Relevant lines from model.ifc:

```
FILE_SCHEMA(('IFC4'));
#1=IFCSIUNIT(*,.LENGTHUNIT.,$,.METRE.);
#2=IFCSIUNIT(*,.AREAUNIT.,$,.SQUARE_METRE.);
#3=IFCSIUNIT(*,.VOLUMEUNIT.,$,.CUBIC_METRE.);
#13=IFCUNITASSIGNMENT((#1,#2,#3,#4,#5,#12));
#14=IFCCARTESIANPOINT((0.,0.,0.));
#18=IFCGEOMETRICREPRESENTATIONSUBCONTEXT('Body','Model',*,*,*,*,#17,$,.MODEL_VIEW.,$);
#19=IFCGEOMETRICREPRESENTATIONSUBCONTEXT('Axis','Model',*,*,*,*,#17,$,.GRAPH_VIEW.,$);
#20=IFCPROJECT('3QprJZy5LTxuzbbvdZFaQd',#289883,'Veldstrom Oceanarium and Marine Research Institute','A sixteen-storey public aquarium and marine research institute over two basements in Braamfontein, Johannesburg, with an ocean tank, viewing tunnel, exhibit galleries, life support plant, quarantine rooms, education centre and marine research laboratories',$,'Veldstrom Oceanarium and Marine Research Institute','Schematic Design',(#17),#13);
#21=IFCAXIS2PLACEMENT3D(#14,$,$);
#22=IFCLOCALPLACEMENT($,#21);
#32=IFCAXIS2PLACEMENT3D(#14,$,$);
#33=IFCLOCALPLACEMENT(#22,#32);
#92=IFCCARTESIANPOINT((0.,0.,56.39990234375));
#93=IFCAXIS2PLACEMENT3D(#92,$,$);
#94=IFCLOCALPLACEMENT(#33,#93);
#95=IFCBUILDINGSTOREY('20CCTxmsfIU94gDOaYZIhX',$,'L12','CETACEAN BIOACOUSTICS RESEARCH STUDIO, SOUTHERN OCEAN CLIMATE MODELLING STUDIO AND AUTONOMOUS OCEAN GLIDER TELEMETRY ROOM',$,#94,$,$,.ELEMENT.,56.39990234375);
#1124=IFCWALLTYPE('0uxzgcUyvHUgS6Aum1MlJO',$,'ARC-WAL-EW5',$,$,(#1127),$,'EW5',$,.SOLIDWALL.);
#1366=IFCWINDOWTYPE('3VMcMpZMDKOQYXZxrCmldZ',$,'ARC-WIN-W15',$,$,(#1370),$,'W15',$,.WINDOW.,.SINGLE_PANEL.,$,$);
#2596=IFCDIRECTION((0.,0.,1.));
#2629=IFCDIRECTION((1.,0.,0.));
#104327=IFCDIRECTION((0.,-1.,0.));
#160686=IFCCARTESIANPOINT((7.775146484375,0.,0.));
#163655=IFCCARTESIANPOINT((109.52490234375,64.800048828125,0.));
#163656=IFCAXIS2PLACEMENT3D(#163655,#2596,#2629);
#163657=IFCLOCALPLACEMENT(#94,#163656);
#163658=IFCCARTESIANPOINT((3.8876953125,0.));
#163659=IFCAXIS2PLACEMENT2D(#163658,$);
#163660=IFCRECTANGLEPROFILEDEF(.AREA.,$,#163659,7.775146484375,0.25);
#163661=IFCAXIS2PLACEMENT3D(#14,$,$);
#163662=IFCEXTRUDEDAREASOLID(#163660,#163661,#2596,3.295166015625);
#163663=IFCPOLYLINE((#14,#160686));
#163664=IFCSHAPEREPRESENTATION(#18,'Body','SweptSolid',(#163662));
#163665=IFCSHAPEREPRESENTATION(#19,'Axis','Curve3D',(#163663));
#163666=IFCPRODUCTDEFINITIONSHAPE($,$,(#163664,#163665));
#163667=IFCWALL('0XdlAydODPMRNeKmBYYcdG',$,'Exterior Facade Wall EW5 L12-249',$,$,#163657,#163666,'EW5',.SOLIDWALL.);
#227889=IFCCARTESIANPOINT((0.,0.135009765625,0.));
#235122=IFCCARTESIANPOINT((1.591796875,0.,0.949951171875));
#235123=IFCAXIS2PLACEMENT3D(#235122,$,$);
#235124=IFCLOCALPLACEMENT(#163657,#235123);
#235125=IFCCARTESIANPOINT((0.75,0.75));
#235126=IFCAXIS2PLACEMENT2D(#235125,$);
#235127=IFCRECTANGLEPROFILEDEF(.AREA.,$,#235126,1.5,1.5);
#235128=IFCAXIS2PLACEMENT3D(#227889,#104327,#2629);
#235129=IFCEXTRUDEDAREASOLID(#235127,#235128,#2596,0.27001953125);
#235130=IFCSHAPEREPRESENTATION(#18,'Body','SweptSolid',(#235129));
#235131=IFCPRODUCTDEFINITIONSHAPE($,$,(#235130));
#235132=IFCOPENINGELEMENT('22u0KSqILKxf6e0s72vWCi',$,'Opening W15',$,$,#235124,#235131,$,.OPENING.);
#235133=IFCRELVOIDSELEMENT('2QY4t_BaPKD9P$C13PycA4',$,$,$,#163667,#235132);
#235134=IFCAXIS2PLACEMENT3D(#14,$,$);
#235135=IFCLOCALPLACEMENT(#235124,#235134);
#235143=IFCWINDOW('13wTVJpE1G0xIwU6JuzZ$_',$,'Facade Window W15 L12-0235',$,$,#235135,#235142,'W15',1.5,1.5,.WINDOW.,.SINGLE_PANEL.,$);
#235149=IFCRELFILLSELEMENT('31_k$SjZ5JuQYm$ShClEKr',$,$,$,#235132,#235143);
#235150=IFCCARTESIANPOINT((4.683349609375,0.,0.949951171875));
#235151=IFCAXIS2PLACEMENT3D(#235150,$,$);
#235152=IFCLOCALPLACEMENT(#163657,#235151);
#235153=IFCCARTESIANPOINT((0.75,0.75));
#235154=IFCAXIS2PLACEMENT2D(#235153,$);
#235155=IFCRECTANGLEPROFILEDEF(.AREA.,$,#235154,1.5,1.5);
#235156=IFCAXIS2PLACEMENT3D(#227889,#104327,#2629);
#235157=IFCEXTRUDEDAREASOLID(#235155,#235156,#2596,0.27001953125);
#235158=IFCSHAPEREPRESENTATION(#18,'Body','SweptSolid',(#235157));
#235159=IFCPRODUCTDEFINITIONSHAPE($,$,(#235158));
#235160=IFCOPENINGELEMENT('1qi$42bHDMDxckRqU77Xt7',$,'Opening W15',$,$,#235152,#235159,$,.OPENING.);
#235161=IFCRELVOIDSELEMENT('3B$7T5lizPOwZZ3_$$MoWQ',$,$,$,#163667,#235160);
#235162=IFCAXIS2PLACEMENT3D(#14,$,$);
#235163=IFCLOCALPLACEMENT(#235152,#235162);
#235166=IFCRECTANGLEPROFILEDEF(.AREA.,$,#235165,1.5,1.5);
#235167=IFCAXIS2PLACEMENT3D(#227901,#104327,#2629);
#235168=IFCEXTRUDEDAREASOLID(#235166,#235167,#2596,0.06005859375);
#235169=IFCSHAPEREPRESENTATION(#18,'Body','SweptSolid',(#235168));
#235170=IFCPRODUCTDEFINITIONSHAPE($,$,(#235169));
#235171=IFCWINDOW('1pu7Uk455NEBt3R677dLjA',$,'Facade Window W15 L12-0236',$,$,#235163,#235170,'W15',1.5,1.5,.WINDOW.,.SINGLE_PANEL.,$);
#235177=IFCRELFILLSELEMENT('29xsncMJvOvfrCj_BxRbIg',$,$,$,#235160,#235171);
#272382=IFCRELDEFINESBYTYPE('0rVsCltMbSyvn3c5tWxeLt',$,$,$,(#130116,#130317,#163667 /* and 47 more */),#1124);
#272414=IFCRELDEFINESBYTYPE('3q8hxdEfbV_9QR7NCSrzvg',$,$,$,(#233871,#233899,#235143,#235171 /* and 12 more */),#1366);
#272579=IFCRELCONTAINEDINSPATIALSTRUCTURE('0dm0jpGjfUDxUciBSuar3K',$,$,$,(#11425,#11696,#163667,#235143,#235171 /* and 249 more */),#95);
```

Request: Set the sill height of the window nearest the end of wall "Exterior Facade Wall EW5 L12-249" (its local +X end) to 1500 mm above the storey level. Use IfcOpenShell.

```python
import numpy as np
import ifcopenshell
import ifcopenshell.api.geometry
import ifcopenshell.geom
import ifcopenshell.util.element
import ifcopenshell.util.placement
import ifcopenshell.util.shape
import ifcopenshell.util.unit

model = ifcopenshell.open("model.ifc")
unit_scale = ifcopenshell.util.unit.calculate_unit_scale(model)

window = model.by_guid("1pu7Uk455NEBt3R677dLjA")
opening = window.FillsVoids[0].RelatingOpeningElement
storey = ifcopenshell.util.element.get_container(window, ifc_class="IfcBuildingStorey")
level = ifcopenshell.util.placement.get_local_placement(storey.ObjectPlacement)[2, 3]

# The opening's origin need not be at the sill, so measure its lowest point.
shape = ifcopenshell.geom.create_shape(ifcopenshell.geom.settings(), opening)
bottom = ifcopenshell.util.shape.get_shape_bottom_elevation(shape, shape.geometry) / unit_scale
dz = level + 1.5 / unit_scale - bottom

shift = np.array([0.0, 0.0, dz])
# The window is placed relative to its opening, so it follows when the opening moves.
matrix = ifcopenshell.util.placement.get_local_placement(opening.ObjectPlacement)
matrix[:3, 3] += shift
ifcopenshell.api.geometry.edit_object_placement(
    model, product=opening, matrix=matrix, is_si=False, should_transform_children=True
)

print(f"moved by {dz * unit_scale:+.3f} m")

model.write("model_edited.ifc")
```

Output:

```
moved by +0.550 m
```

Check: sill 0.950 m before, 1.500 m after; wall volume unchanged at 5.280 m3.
